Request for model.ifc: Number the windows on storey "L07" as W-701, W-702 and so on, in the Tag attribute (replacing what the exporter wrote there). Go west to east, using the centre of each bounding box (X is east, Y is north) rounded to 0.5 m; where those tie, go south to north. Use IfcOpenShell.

First a look at what the model holds.

```python
import ifcopenshell
import ifcopenshell.util.element
import ifcopenshell.util.placement

model = ifcopenshell.open("model.ifc")
print(model.schema)
storey = next(s for s in model.by_type("IfcBuildingStorey") if s.Name == "L07")
windows = [e for e in ifcopenshell.util.element.get_decomposition(storey) if e.is_a("IfcWindow")]
for e in sorted(windows, key=lambda e: e.id()):
    origin = ifcopenshell.util.placement.get_local_placement(e.ObjectPlacement)[:3, 3]
    print(e.id(), e.Tag, e.Name, origin.round(2) + 0.0, sep=" | ")
```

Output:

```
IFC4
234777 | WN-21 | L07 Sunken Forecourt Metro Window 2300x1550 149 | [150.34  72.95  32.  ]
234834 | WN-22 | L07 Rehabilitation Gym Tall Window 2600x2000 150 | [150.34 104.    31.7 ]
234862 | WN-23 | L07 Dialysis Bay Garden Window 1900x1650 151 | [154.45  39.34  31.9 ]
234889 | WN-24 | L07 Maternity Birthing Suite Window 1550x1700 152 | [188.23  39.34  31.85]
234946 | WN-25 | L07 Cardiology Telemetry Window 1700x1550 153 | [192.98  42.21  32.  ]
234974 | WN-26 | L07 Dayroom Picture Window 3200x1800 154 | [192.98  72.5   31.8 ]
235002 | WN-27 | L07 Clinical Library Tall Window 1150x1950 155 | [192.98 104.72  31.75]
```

```python
import ifcopenshell
import ifcopenshell.geom
import ifcopenshell.util.element
import ifcopenshell.util.shape

model = ifcopenshell.open("model.ifc")
settings = ifcopenshell.geom.settings()
settings.set("use-world-coords", True)


def centre(element):
    shape = ifcopenshell.geom.create_shape(settings, element)
    return ifcopenshell.util.shape.get_bbox_centroid(shape.geometry)


storey = next(s for s in model.by_type("IfcBuildingStorey") if s.Name == "L07")
windows = [e for e in ifcopenshell.util.element.get_decomposition(storey) if e.is_a("IfcWindow")]

# Insertion points can sit at a corner or the storey origin, so sort by the geometry (in metres).
centres = {e: centre(e) for e in windows}
windows.sort(key=lambda e: (round(centres[e][0] / 0.5), centres[e][1]))

for i, e in enumerate(windows, start=1):
    number = f"W-7{i:02d}"
    e.Tag = number
    print(e.id(), number)

model.write("model_v2.ifc")
```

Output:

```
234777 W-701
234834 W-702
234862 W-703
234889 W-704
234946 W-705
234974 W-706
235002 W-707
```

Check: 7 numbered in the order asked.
